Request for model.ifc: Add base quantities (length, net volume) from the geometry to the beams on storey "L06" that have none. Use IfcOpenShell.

First a look at what the model holds.

```python
import ifcopenshell
import ifcopenshell.util.element
import ifcopenshell.util.unit

model = ifcopenshell.open("model.ifc")
print(model.schema)
for unit_type in ("LENGTHUNIT", "AREAUNIT", "VOLUMEUNIT"):
    print(unit_type, ifcopenshell.util.unit.calculate_unit_scale(model, unit_type))
storey = next(s for s in model.by_type("IfcBuildingStorey") if s.Name == "L06")
beams = [e for e in ifcopenshell.util.element.get_decomposition(storey) if e.is_a("IfcBeam")]
for e in sorted(beams, key=lambda e: e.id()):
    print(e.id(), e.is_a(), e.Name, list(ifcopenshell.util.element.get_psets(e, qtos_only=True)), sep=" | ")
```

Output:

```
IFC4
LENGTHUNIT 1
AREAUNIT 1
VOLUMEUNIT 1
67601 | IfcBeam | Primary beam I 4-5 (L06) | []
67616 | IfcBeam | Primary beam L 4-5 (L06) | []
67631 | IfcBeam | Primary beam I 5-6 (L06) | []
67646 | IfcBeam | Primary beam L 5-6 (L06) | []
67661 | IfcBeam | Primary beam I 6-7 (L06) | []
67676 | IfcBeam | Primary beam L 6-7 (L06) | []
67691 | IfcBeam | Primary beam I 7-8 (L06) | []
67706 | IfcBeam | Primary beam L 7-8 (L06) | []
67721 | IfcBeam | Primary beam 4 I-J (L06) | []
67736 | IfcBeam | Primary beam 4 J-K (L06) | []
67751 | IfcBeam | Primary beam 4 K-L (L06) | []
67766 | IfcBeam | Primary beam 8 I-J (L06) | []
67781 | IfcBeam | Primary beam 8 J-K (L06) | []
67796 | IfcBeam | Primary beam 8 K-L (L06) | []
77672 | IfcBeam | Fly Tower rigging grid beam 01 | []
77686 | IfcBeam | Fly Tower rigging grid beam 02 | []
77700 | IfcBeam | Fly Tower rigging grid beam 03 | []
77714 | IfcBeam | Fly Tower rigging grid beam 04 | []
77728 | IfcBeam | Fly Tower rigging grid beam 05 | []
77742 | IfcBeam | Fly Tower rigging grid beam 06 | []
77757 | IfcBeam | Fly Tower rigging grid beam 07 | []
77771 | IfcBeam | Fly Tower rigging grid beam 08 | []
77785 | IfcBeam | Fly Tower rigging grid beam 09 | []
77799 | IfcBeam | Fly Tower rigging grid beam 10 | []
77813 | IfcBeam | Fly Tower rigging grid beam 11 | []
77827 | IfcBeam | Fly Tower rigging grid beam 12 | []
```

```python
import ifcopenshell
import ifcopenshell.api.pset
import ifcopenshell.geom
import ifcopenshell.util.element
import ifcopenshell.util.shape
import ifcopenshell.util.unit

model = ifcopenshell.open("model.ifc")
unit_scale = ifcopenshell.util.unit.calculate_unit_scale(model)
volume_scale = ifcopenshell.util.unit.calculate_unit_scale(model, "VOLUMEUNIT")
settings = ifcopenshell.geom.settings()

storey = next(s for s in model.by_type("IfcBuildingStorey") if s.Name == "L06")
beams = [e for e in ifcopenshell.util.element.get_decomposition(storey) if e.is_a("IfcBeam")]

for e in sorted(beams, key=lambda e: e.id()):
    if ifcopenshell.util.element.get_psets(e, qtos_only=True, should_inherit=False):
        continue
    # Geometry comes back in metres, in the element's own axes.
    shape = ifcopenshell.geom.create_shape(settings, e)
    values = {
        "Length": ifcopenshell.util.shape.get_max_xyz(shape.geometry) / unit_scale,
        "NetVolume": ifcopenshell.util.shape.get_volume(shape.geometry) / volume_scale,
    }
    qto = ifcopenshell.api.pset.add_qto(model, product=e, name="Qto_BeamBaseQuantities")
    ifcopenshell.api.pset.edit_qto(model, qto=qto, properties=values)
    print(e.id(), {k: round(v, 3) for k, v in values.items()})

model.write("model_edited.ifc")
```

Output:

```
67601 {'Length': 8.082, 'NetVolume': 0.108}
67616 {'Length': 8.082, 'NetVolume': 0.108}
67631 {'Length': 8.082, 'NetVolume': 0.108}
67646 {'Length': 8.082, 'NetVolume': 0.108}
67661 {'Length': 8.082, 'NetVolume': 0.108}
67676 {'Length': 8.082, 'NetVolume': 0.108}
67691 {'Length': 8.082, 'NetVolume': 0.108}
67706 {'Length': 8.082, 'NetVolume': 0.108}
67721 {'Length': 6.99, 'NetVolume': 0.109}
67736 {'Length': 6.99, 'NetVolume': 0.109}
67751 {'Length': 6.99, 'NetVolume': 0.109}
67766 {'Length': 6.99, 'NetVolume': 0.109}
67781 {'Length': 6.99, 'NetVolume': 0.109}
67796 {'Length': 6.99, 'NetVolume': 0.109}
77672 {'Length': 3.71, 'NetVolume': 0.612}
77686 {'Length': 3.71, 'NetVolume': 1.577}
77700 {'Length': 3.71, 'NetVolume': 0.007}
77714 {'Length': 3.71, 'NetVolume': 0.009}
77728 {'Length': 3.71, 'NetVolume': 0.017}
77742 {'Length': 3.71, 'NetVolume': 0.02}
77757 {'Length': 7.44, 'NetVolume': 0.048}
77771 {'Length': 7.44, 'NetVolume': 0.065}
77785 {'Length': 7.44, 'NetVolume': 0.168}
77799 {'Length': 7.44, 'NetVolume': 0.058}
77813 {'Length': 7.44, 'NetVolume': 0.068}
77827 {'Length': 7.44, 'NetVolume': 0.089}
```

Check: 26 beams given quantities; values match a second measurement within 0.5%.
